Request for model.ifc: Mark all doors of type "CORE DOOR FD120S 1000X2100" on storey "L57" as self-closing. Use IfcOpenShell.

First a look at what the model holds.

```python
import ifcopenshell
import ifcopenshell.util.element

model = ifcopenshell.open("model.ifc")
print(model.schema)
storey = next(s for s in model.by_type("IfcBuildingStorey") if s.Name == "L57")
doors = [e for e in ifcopenshell.util.element.get_decomposition(storey) if e.is_a("IfcDoor")]
seen = {}
for e in doors:
    element_type = ifcopenshell.util.element.get_type(e)
    key = (element_type.Name if element_type != e and element_type else None, ifcopenshell.util.element.get_pset(e, "Pset_DoorCommon", "SelfClosing"))
    seen[key] = seen.get(key, 0) + 1
for (name, value), count in sorted(seen.items(), key=str):
    print(count, "x", name, "|", value)
```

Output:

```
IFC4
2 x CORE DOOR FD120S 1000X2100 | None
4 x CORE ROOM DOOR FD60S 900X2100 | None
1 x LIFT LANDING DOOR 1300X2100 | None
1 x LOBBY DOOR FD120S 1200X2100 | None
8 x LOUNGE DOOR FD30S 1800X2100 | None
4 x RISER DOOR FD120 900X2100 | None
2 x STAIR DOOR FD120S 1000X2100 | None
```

```python
import ifcopenshell
import ifcopenshell.api.pset
import ifcopenshell.util.element

model = ifcopenshell.open("model.ifc")

storey = next(s for s in model.by_type("IfcBuildingStorey") if s.Name == "L57")
doors = [e for e in ifcopenshell.util.element.get_decomposition(storey) if e.is_a("IfcDoor")]

count = 0
for e in doors:
    element_type = ifcopenshell.util.element.get_type(e)
    if element_type in (None, e) or element_type.Name != "CORE DOOR FD120S 1000X2100":
        continue
    found = ifcopenshell.util.element.get_pset(e, "Pset_DoorCommon", should_inherit=False)
    if found:
        pset = model.by_id(found["id"])
        if len(ifcopenshell.util.element.get_elements_by_pset(pset)) > 1:
            pset = ifcopenshell.api.pset.unshare_pset(model, products=[e], pset=pset)[0]
    else:
        pset = ifcopenshell.api.pset.add_pset(model, product=e, name="Pset_DoorCommon")
    ifcopenshell.api.pset.edit_pset(model, pset=pset, properties={"SelfClosing": True})
    count += 1

print(count, "doors updated")

model.write("model_v2.ifc")
```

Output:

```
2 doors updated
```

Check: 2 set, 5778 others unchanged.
